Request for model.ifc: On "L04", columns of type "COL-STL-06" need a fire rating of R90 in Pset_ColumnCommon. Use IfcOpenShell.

First a look at what the model holds.

```python
import ifcopenshell
import ifcopenshell.util.element

model = ifcopenshell.open("model.ifc")
print(model.schema)
storey = next(s for s in model.by_type("IfcBuildingStorey") if s.Name == "L04")
columns = [e for e in ifcopenshell.util.element.get_decomposition(storey) if e.is_a("IfcColumn")]
seen = {}
for e in columns:
    element_type = ifcopenshell.util.element.get_type(e)
    key = (element_type.Name if element_type != e and element_type else None, ifcopenshell.util.element.get_pset(e, "Pset_ColumnCommon", "FireRating"))
    seen[key] = seen.get(key, 0) + 1
for (name, value), count in sorted(seen.items(), key=str):
    print(count, "x", name, "|", value)
```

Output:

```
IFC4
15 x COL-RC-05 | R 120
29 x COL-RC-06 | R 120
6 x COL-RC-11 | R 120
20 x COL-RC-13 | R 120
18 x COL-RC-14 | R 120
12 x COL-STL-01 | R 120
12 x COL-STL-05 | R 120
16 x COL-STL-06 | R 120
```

```python
import ifcopenshell
import ifcopenshell.api.pset
import ifcopenshell.util.element

model = ifcopenshell.open("model.ifc")

storey = next(s for s in model.by_type("IfcBuildingStorey") if s.Name == "L04")
columns = [e for e in ifcopenshell.util.element.get_decomposition(storey) if e.is_a("IfcColumn")]

count = 0
for e in columns:
    element_type = ifcopenshell.util.element.get_type(e)
    if element_type in (None, e) or element_type.Name != "COL-STL-06":
        continue
    # add_pset returns the element's existing set when there is one.
    pset = ifcopenshell.api.pset.add_pset(model, product=e, name="Pset_ColumnCommon")
    ifcopenshell.api.pset.edit_pset(model, pset=pset, properties={"FireRating": "R90"})
    count += 1

print(count, "columns updated")

model.write("model_rev.ifc")
```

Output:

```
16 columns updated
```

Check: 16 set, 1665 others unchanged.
